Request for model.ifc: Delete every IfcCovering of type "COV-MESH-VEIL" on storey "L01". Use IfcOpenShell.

First a look at what the model holds.

```python
import ifcopenshell
import ifcopenshell.util.element

model = ifcopenshell.open("model.ifc")
print(model.schema)
storey = next(s for s in model.by_type("IfcBuildingStorey") if s.Name == "L01")
coverings = [e for e in ifcopenshell.util.element.get_decomposition(storey) if e.is_a("IfcCovering")]
seen = {}
for e in coverings:
    element_type = ifcopenshell.util.element.get_type(e)
    name = element_type.Name if element_type not in (None, e) else None
    seen[name] = seen.get(name, 0) + 1
for name, count in sorted(seen.items(), key=str):
    print(count, "x", name)
```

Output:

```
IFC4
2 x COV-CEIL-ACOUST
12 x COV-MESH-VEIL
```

```python
import ifcopenshell
import ifcopenshell.api.root
import ifcopenshell.util.element

model = ifcopenshell.open("model.ifc")

storey = next(s for s in model.by_type("IfcBuildingStorey") if s.Name == "L01")
coverings = [e for e in ifcopenshell.util.element.get_decomposition(storey) if e.is_a("IfcCovering")]
targets = [e for e in coverings if (t := ifcopenshell.util.element.get_type(e)) not in (None, e) and t.Name == "COV-MESH-VEIL"]

for e in targets:
    ifcopenshell.api.root.remove_product(model, product=e)
print(len(targets), "removed")

model.write("model_rev.ifc")
```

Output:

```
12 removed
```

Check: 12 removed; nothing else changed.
